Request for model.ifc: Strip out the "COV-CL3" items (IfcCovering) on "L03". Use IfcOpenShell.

First a look at what the model holds.

```python
import ifcopenshell
import ifcopenshell.util.element

model = ifcopenshell.open("model.ifc")
print(model.schema)
storey = next(s for s in model.by_type("IfcBuildingStorey") if s.Name == "L03")
coverings = [e for e in ifcopenshell.util.element.get_decomposition(storey) if e.is_a("IfcCovering")]
seen = {}
for e in coverings:
    element_type = ifcopenshell.util.element.get_type(e)
    name = element_type.Name if element_type not in (None, e) else None
    seen[name] = seen.get(name, 0) + 1
for name, count in sorted(seen.items(), key=str):
    print(count, "x", name)
```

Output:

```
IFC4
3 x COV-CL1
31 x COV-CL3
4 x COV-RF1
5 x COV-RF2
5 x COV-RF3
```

```python
import ifcopenshell
import ifcopenshell.api.root
import ifcopenshell.util.element

model = ifcopenshell.open("model.ifc")

storey = next(s for s in model.by_type("IfcBuildingStorey") if s.Name == "L03")
coverings = [e for e in ifcopenshell.util.element.get_decomposition(storey) if e.is_a("IfcCovering")]
targets = [e for e in coverings if (t := ifcopenshell.util.element.get_type(e)) not in (None, e) and t.Name == "COV-CL3"]

for e in targets:
    ifcopenshell.api.root.remove_product(model, product=e)
print(len(targets), "removed")

model.write("model_edited.ifc")
```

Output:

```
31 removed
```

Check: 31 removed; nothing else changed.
